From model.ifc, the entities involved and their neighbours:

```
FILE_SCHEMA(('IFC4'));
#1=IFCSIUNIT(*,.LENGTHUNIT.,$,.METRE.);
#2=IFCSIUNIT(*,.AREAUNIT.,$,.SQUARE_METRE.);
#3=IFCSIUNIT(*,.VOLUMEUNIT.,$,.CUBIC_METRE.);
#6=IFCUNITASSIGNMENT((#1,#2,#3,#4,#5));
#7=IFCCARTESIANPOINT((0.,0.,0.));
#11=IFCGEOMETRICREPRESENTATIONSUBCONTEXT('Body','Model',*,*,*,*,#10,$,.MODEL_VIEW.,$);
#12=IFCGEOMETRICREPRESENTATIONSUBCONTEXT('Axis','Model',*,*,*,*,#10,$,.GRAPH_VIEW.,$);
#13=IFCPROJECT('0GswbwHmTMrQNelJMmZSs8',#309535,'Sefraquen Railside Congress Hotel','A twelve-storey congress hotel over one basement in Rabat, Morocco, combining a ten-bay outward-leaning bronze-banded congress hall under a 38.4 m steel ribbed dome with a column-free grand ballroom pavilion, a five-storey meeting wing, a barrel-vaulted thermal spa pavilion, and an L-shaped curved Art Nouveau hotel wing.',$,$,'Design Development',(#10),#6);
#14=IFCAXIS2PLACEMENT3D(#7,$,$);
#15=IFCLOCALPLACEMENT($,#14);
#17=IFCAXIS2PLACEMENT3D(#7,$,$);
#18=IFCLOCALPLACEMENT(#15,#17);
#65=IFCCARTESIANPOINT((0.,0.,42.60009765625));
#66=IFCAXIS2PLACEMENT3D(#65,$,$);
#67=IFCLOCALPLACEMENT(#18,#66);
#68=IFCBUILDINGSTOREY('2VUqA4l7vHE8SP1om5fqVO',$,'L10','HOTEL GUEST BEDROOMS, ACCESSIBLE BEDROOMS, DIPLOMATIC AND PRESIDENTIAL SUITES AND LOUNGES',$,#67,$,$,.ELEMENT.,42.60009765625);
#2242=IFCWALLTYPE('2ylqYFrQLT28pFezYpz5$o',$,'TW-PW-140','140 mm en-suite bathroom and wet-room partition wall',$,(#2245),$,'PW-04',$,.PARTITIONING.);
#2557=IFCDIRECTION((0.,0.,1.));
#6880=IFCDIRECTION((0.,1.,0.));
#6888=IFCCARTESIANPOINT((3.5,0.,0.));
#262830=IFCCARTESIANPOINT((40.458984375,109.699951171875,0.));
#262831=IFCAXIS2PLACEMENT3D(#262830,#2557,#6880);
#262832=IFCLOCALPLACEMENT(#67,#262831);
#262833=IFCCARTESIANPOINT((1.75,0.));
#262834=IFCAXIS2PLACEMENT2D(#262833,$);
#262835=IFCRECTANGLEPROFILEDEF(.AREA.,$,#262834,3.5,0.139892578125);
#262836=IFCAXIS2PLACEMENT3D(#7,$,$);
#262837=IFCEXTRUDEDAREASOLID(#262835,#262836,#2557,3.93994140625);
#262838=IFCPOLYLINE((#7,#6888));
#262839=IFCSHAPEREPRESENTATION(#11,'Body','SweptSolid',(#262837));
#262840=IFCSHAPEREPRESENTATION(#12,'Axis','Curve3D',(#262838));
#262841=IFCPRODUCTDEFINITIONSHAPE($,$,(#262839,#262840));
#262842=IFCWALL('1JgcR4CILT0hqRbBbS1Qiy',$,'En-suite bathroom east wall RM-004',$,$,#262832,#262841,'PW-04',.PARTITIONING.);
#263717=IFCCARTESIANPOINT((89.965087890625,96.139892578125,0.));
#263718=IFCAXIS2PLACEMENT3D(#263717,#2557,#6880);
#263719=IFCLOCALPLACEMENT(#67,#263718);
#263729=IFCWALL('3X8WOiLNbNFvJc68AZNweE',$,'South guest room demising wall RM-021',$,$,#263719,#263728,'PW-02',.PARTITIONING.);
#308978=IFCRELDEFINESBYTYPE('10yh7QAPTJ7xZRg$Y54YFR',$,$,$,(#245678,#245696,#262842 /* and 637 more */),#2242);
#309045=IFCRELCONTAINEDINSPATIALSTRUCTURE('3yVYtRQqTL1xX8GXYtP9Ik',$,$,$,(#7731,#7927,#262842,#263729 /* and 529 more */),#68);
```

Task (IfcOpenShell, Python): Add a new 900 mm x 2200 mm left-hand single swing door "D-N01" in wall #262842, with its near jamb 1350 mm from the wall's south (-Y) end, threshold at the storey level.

```python
import numpy as np
import ifcopenshell
import ifcopenshell.api.feature
import ifcopenshell.api.geometry
import ifcopenshell.api.root
import ifcopenshell.api.spatial
import ifcopenshell.geom
import ifcopenshell.util.element
import ifcopenshell.util.placement
import ifcopenshell.util.representation
import ifcopenshell.util.shape
import ifcopenshell.util.unit

model = ifcopenshell.open("model.ifc")
unit_scale = ifcopenshell.util.unit.calculate_unit_scale(model)
settings = ifcopenshell.geom.settings()


def volume(element):
    """Net volume in cubic metres, openings subtracted."""
    shape = ifcopenshell.geom.create_shape(settings, element)
    return ifcopenshell.util.shape.get_volume(shape.geometry)


wall = model.by_guid("1JgcR4CILT0hqRbBbS1Qiy")
storey = ifcopenshell.util.element.get_container(wall, ifc_class="IfcBuildingStorey")
context = ifcopenshell.util.representation.get_context(model, "Model", "Body", "MODEL_VIEW")
before = volume(wall)

width, height, from_end, sill = 0.9, 2.2, 1.35, 0.0  # metres

# The wall runs along its own X axis, and the end named is its -X end.
wall_shape = ifcopenshell.geom.create_shape(settings, wall)
x, y, z = ifcopenshell.util.shape.get_vertices(wall_shape.geometry).T
start = x.min() + from_end
face, thickness = float(y.min()), float(y.max() - y.min())
wall_matrix = ifcopenshell.util.placement.get_local_placement(wall.ObjectPlacement)
level = ifcopenshell.util.placement.get_local_placement(storey.ObjectPlacement)[2, 3]


def in_wall(x, y):
    """Placement at x, y metres in the wall's axes, at sill height."""
    matrix = wall_matrix.copy()
    matrix[:, 3] = wall_matrix @ np.array([x / unit_scale, y / unit_scale, 0.0, 1.0])
    matrix[2, 3] = level + sill / unit_scale
    return matrix


# Opening: a box that overshoots both wall faces by 50 mm.
opening = ifcopenshell.api.root.create_entity(model, ifc_class="IfcOpeningElement", predefined_type="OPENING")
box = ifcopenshell.api.geometry.add_wall_representation(
    model, context=context, length=width, height=height, thickness=thickness + 0.1
)
ifcopenshell.api.geometry.assign_representation(model, product=opening, representation=box)
ifcopenshell.api.geometry.edit_object_placement(model, product=opening, matrix=in_wall(start, face - 0.05), is_si=False)
ifcopenshell.api.feature.add_feature(model, feature=opening, element=wall)

door = ifcopenshell.api.root.create_entity(model, ifc_class="IfcDoor", name="D-N01", predefined_type="DOOR")
door.OverallWidth, door.OverallHeight = width / unit_scale, height / unit_scale
door.OperationType = "SINGLE_SWING_LEFT"
body = ifcopenshell.api.geometry.add_door_representation(
    model,
    context=context,
    overall_width=door.OverallWidth,
    overall_height=door.OverallHeight,
    operation_type="SINGLE_SWING_LEFT",
    lining_properties={"LiningDepth": thickness / unit_scale, "ThresholdDepth": thickness / unit_scale},
)
ifcopenshell.api.geometry.assign_representation(model, product=door, representation=body)
ifcopenshell.api.spatial.assign_container(model, products=[door], relating_structure=storey)
ifcopenshell.api.feature.add_filling(model, opening=opening, element=door)

# The lining spans the wall, so the door starts at the wall face.
ifcopenshell.api.geometry.edit_object_placement(model, product=door, matrix=in_wall(start, face), is_si=False)

after = volume(wall)

print(f"wall volume {before:.3f} -> {after:.3f} m3")

model.write("model_v2.ifc")
```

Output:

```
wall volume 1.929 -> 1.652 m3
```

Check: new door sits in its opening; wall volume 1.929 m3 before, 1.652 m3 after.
